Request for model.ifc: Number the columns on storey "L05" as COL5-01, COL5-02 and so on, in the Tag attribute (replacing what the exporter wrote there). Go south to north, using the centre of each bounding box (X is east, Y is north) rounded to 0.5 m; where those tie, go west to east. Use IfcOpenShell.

First a look at what the model holds.

```python
import ifcopenshell
import ifcopenshell.util.element
import ifcopenshell.util.placement

model = ifcopenshell.open("model.ifc")
print(model.schema)
storey = next(s for s in model.by_type("IfcBuildingStorey") if s.Name == "L05")
columns = [e for e in ifcopenshell.util.element.get_decomposition(storey) if e.is_a("IfcColumn")]
for e in sorted(columns, key=lambda e: e.id()):
    origin = ifcopenshell.util.placement.get_local_placement(e.ObjectPlacement)[:3, 3]
    print(e.id(), e.Tag, e.Name, origin.round(2) + 0.0, sep=" | ")
```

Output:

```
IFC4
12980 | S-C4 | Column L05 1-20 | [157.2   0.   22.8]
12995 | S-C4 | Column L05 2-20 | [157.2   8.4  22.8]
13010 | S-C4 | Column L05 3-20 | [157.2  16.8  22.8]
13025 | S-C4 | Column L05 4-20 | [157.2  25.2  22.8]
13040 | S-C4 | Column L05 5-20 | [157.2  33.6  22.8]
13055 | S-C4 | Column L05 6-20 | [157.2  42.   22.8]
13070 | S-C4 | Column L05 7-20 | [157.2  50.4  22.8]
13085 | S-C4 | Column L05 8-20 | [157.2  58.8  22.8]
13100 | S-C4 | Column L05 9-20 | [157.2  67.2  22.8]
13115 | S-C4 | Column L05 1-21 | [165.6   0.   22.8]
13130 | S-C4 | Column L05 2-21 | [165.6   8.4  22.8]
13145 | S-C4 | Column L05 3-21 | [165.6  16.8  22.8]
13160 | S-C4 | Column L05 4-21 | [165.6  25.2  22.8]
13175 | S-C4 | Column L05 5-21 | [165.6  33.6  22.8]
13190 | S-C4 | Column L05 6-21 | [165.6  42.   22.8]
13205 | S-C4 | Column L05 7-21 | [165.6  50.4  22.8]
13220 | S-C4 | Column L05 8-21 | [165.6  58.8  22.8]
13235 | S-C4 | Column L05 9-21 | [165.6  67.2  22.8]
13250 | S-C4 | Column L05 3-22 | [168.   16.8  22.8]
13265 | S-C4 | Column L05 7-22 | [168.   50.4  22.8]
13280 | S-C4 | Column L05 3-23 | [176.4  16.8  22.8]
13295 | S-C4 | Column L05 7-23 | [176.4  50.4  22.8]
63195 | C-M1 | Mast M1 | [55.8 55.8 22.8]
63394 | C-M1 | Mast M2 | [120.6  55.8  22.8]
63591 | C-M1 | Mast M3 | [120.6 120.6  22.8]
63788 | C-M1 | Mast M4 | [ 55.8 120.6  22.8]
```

```python
import ifcopenshell
import ifcopenshell.geom
import ifcopenshell.util.element
import ifcopenshell.util.shape

model = ifcopenshell.open("model.ifc")
settings = ifcopenshell.geom.settings()
settings.set("use-world-coords", True)


def centre(element):
    shape = ifcopenshell.geom.create_shape(settings, element)
    return ifcopenshell.util.shape.get_bbox_centroid(shape.geometry)


storey = next(s for s in model.by_type("IfcBuildingStorey") if s.Name == "L05")
columns = [e for e in ifcopenshell.util.element.get_decomposition(storey) if e.is_a("IfcColumn")]

# Insertion points can sit at a corner or the storey origin, so sort by the geometry (in metres).
centres = {e: centre(e) for e in columns}
columns.sort(key=lambda e: (round(centres[e][1] / 0.5), centres[e][0]))

for i, e in enumerate(columns, start=1):
    number = f"COL5-{i:02d}"
    e.Tag = number
    print(e.id(), number)

model.write("model_edited.ifc")
```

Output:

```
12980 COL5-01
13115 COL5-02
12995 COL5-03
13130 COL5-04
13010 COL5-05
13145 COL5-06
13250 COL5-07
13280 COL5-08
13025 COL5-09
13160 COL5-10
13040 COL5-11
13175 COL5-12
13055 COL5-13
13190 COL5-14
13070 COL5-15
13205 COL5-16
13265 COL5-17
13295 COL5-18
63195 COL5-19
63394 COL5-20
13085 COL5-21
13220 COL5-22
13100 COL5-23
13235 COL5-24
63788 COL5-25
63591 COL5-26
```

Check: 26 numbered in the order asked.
